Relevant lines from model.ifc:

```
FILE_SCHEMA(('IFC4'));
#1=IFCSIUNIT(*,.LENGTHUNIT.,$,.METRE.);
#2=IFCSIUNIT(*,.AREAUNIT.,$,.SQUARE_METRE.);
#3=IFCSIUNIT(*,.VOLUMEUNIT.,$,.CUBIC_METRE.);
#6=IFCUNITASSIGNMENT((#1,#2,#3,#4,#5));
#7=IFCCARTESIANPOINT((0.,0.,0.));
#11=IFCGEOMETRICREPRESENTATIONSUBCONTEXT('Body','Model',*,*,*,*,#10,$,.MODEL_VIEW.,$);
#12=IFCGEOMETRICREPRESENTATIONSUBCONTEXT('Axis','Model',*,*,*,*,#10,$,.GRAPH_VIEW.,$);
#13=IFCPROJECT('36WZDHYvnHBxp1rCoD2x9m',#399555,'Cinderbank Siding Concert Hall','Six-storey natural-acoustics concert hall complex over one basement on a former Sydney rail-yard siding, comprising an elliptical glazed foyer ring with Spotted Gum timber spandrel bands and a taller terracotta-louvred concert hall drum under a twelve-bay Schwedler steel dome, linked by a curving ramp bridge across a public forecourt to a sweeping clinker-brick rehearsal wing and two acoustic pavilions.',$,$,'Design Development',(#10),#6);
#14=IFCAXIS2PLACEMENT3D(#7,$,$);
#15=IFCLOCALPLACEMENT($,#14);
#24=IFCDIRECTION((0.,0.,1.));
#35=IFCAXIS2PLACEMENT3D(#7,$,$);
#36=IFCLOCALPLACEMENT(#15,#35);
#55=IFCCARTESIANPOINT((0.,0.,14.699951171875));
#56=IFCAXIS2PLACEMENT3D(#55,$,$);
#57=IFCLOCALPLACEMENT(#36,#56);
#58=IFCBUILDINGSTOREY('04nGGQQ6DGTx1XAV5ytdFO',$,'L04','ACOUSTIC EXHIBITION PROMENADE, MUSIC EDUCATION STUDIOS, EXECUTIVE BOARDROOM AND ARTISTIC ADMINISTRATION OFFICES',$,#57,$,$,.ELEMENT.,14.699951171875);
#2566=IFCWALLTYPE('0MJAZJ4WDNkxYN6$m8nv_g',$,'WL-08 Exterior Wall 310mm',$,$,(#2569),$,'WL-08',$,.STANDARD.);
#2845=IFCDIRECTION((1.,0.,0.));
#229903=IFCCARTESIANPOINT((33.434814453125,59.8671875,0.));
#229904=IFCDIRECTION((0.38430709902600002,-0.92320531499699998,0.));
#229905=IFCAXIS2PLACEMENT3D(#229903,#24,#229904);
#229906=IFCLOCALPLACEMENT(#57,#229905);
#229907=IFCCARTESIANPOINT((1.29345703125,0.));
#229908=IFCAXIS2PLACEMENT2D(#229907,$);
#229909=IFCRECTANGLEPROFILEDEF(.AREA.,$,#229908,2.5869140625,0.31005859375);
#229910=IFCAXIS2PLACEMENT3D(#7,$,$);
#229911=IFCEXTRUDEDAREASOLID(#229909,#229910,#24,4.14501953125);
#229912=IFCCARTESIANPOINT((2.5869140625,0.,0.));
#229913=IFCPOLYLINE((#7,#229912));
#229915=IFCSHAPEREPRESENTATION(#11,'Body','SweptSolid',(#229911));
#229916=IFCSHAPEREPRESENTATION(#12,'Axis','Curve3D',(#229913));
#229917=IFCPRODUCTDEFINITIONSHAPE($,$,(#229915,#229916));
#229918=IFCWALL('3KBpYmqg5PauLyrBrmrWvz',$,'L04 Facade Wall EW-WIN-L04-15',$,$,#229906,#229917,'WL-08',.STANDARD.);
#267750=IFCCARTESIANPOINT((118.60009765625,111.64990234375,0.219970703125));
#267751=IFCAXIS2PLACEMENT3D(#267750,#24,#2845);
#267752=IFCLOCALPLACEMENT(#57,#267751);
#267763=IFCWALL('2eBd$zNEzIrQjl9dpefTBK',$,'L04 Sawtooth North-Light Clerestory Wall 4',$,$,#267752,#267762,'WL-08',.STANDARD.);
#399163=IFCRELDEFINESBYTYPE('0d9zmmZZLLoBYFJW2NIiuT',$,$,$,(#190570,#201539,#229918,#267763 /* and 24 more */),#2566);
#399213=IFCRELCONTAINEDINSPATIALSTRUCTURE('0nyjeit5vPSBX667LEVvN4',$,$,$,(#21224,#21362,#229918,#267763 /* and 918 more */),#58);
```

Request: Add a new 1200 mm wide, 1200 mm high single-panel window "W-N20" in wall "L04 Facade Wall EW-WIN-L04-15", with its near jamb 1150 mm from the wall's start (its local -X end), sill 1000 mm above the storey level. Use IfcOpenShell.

```python
import numpy as np
import ifcopenshell
import ifcopenshell.api.feature
import ifcopenshell.api.geometry
import ifcopenshell.api.root
import ifcopenshell.api.spatial
import ifcopenshell.geom
import ifcopenshell.util.element
import ifcopenshell.util.placement
import ifcopenshell.util.representation
import ifcopenshell.util.shape
import ifcopenshell.util.unit

model = ifcopenshell.open("model.ifc")
unit_scale = ifcopenshell.util.unit.calculate_unit_scale(model)
settings = ifcopenshell.geom.settings()


def volume(element):
    """Net volume in cubic metres, openings subtracted."""
    shape = ifcopenshell.geom.create_shape(settings, element)
    return ifcopenshell.util.shape.get_volume(shape.geometry)


wall = model.by_id(229918)
storey = ifcopenshell.util.element.get_container(wall, ifc_class="IfcBuildingStorey")
context = ifcopenshell.util.representation.get_context(model, "Model", "Body", "MODEL_VIEW")
before = volume(wall)

width, height, from_end, sill = 1.2, 1.2, 1.15, 1  # metres

# The wall runs along its own X axis, and the end named is its -X end.
wall_shape = ifcopenshell.geom.create_shape(settings, wall)
x, y, z = ifcopenshell.util.shape.get_vertices(wall_shape.geometry).T
start = x.min() + from_end
face, thickness = float(y.min()), float(y.max() - y.min())
wall_matrix = ifcopenshell.util.placement.get_local_placement(wall.ObjectPlacement)
level = ifcopenshell.util.placement.get_local_placement(storey.ObjectPlacement)[2, 3]


def in_wall(x, y):
    """Placement at x, y metres in the wall's axes, at sill height."""
    matrix = wall_matrix.copy()
    matrix[:, 3] = wall_matrix @ np.array([x / unit_scale, y / unit_scale, 0.0, 1.0])
    matrix[2, 3] = level + sill / unit_scale
    return matrix


# Opening: a box that overshoots both wall faces by 50 mm.
opening = ifcopenshell.api.root.create_entity(model, ifc_class="IfcOpeningElement", predefined_type="OPENING")
box = ifcopenshell.api.geometry.add_wall_representation(
    model, context=context, length=width, height=height, thickness=thickness + 0.1
)
ifcopenshell.api.geometry.assign_representation(model, product=opening, representation=box)
ifcopenshell.api.geometry.edit_object_placement(model, product=opening, matrix=in_wall(start, face - 0.05), is_si=False)
ifcopenshell.api.feature.add_feature(model, feature=opening, element=wall)

window = ifcopenshell.api.root.create_entity(model, ifc_class="IfcWindow", name="W-N20", predefined_type="WINDOW")
window.OverallWidth, window.OverallHeight = width / unit_scale, height / unit_scale
window.PartitioningType = "SINGLE_PANEL"
body = ifcopenshell.api.geometry.add_window_representation(
    model,
    context=context,
    overall_width=window.OverallWidth,
    overall_height=window.OverallHeight,
    partition_type="SINGLE_PANEL",
)
ifcopenshell.api.geometry.assign_representation(model, product=window, representation=body)
ifcopenshell.api.spatial.assign_container(model, products=[window], relating_structure=storey)
ifcopenshell.api.feature.add_filling(model, opening=opening, element=window)

# Centre the window in the wall's thickness.
ifcopenshell.api.geometry.edit_object_placement(model, product=window, matrix=in_wall(start, face), is_si=False)
window_shape = ifcopenshell.geom.create_shape(settings, window)
depth = ifcopenshell.util.shape.get_vertices(window_shape.geometry)[:, 1]
offset = face + thickness / 2 - (depth.min() + depth.max()) / 2
ifcopenshell.api.geometry.edit_object_placement(model, product=window, matrix=in_wall(start, offset), is_si=False)

after = volume(wall)

print(f"wall volume {before:.3f} -> {after:.3f} m3")

model.write("model_rev.ifc")
```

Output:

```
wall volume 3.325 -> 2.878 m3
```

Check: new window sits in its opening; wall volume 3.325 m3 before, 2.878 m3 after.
